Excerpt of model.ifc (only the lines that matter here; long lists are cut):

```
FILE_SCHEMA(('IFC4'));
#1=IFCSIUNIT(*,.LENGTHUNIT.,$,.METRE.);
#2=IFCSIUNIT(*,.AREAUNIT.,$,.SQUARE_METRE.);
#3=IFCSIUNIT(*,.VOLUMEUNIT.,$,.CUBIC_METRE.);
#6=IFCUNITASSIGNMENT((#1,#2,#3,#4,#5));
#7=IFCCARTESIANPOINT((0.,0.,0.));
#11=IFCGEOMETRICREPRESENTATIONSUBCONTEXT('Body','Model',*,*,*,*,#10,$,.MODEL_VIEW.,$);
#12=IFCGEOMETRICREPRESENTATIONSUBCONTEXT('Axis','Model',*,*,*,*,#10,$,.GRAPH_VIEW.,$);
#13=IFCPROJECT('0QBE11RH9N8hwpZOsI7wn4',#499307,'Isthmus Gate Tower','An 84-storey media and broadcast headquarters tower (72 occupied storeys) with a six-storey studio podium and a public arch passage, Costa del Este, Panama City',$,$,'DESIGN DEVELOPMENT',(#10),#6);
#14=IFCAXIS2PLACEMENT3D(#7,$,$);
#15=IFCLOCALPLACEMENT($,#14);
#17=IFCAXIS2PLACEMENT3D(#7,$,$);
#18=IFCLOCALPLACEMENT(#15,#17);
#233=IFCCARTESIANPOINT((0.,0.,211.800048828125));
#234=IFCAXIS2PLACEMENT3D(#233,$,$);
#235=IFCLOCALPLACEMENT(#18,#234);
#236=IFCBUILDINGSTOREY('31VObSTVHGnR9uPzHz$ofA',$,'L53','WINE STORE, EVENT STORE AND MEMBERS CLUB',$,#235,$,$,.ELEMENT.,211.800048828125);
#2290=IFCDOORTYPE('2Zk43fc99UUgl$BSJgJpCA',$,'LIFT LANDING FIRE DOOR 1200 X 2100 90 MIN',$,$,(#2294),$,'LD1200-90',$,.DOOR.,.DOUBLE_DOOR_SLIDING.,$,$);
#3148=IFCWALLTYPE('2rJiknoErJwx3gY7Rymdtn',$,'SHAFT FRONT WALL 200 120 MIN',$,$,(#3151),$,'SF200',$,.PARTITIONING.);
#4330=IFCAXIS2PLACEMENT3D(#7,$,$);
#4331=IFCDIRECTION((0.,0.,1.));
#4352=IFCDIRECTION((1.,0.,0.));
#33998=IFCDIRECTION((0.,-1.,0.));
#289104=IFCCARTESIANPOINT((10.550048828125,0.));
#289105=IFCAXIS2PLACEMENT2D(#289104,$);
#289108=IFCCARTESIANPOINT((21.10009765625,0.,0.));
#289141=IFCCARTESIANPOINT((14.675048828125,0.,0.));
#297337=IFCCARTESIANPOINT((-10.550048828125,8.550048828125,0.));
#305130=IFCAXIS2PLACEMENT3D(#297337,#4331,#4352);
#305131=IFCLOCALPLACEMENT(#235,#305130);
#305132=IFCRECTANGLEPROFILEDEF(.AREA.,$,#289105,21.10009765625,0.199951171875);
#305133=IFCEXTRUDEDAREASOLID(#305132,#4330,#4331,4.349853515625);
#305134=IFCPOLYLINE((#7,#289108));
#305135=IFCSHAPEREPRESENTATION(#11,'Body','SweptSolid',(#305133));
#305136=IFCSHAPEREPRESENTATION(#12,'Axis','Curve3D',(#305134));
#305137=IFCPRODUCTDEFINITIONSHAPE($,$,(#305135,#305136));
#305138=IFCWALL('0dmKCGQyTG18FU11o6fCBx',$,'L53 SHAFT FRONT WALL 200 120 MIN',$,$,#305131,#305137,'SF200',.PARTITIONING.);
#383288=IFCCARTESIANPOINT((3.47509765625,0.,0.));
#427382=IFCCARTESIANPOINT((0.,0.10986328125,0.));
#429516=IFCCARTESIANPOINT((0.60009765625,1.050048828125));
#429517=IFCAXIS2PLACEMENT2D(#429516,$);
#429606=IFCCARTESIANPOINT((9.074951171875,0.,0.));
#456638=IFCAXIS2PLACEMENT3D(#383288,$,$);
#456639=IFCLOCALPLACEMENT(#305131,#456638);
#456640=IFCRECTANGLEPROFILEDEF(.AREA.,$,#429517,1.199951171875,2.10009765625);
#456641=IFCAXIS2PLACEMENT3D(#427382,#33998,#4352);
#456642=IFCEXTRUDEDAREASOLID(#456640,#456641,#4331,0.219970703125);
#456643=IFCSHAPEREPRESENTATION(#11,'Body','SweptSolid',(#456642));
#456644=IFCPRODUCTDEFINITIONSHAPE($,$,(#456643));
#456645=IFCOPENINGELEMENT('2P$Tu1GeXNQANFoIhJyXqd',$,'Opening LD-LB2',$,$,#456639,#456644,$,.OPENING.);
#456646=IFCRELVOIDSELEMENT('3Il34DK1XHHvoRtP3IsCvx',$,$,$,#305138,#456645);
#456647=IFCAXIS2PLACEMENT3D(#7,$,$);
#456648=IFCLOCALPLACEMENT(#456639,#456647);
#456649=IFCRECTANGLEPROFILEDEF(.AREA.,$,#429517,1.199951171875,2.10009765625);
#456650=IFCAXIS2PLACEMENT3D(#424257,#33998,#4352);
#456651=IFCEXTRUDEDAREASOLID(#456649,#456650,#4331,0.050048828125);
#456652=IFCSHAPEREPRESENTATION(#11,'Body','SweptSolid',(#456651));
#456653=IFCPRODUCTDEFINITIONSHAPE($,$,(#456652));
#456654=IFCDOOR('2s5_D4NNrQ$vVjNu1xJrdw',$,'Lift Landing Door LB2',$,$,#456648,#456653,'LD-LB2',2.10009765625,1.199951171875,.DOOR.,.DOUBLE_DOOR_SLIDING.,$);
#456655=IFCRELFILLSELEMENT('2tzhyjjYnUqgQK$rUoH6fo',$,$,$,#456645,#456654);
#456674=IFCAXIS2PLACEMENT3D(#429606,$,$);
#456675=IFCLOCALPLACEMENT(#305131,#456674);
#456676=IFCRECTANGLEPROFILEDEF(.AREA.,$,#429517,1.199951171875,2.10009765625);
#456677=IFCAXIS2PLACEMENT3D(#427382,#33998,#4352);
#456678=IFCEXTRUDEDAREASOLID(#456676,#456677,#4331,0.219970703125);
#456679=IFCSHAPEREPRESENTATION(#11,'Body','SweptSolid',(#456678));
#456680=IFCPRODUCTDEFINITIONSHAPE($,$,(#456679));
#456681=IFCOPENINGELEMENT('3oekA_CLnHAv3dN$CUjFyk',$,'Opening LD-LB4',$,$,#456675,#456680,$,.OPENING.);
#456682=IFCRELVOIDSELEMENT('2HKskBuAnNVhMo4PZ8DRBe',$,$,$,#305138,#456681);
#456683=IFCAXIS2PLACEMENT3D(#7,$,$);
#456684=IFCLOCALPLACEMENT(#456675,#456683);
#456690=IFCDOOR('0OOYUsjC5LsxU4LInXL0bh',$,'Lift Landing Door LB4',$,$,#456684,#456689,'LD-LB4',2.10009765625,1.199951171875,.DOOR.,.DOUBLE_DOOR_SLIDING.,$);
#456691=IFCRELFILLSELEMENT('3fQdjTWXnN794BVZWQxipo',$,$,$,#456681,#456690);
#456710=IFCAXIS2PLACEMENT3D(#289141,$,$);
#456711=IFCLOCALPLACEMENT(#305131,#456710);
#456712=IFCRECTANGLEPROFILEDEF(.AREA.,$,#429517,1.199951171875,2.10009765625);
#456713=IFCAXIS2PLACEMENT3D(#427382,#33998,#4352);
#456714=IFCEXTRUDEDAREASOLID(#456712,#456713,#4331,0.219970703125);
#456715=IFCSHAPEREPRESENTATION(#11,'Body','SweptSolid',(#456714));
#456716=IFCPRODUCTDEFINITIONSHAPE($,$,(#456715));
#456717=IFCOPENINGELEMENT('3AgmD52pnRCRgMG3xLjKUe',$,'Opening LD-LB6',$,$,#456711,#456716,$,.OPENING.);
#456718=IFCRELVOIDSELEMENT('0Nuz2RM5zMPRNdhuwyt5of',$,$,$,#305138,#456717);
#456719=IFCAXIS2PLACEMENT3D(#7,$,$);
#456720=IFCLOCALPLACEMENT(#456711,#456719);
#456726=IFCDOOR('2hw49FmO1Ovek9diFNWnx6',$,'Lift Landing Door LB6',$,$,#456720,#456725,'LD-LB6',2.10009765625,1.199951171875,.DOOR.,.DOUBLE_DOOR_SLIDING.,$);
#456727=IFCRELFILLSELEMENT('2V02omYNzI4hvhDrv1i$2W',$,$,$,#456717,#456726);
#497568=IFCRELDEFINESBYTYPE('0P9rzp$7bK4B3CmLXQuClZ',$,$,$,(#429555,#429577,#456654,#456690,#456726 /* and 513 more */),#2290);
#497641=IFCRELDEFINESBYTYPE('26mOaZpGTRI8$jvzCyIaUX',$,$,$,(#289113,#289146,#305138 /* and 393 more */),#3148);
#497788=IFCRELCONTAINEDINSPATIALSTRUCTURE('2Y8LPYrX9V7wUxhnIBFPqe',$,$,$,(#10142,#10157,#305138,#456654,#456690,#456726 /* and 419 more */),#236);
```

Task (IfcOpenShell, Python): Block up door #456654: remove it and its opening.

```python
import ifcopenshell
import ifcopenshell.api.feature
import ifcopenshell.api.root
import ifcopenshell.geom
import ifcopenshell.util.shape

model = ifcopenshell.open("model.ifc")
settings = ifcopenshell.geom.settings()


def volume(element):
    """Net volume in cubic metres, openings subtracted."""
    shape = ifcopenshell.geom.create_shape(settings, element)
    return ifcopenshell.util.shape.get_volume(shape.geometry)


door = model.by_guid("2s5_D4NNrQ$vVjNu1xJrdw")
opening = door.FillsVoids[0].RelatingOpeningElement
wall = opening.VoidsElements[0].RelatingBuildingElement
before = volume(wall)

ifcopenshell.api.root.remove_product(model, product=door)
ifcopenshell.api.feature.remove_feature(model, feature=opening)

after = volume(wall)

print(f"wall volume {before:.3f} -> {after:.3f} m3")

model.write("model-out.ifc")
```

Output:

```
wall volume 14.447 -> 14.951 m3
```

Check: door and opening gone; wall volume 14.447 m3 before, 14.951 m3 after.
